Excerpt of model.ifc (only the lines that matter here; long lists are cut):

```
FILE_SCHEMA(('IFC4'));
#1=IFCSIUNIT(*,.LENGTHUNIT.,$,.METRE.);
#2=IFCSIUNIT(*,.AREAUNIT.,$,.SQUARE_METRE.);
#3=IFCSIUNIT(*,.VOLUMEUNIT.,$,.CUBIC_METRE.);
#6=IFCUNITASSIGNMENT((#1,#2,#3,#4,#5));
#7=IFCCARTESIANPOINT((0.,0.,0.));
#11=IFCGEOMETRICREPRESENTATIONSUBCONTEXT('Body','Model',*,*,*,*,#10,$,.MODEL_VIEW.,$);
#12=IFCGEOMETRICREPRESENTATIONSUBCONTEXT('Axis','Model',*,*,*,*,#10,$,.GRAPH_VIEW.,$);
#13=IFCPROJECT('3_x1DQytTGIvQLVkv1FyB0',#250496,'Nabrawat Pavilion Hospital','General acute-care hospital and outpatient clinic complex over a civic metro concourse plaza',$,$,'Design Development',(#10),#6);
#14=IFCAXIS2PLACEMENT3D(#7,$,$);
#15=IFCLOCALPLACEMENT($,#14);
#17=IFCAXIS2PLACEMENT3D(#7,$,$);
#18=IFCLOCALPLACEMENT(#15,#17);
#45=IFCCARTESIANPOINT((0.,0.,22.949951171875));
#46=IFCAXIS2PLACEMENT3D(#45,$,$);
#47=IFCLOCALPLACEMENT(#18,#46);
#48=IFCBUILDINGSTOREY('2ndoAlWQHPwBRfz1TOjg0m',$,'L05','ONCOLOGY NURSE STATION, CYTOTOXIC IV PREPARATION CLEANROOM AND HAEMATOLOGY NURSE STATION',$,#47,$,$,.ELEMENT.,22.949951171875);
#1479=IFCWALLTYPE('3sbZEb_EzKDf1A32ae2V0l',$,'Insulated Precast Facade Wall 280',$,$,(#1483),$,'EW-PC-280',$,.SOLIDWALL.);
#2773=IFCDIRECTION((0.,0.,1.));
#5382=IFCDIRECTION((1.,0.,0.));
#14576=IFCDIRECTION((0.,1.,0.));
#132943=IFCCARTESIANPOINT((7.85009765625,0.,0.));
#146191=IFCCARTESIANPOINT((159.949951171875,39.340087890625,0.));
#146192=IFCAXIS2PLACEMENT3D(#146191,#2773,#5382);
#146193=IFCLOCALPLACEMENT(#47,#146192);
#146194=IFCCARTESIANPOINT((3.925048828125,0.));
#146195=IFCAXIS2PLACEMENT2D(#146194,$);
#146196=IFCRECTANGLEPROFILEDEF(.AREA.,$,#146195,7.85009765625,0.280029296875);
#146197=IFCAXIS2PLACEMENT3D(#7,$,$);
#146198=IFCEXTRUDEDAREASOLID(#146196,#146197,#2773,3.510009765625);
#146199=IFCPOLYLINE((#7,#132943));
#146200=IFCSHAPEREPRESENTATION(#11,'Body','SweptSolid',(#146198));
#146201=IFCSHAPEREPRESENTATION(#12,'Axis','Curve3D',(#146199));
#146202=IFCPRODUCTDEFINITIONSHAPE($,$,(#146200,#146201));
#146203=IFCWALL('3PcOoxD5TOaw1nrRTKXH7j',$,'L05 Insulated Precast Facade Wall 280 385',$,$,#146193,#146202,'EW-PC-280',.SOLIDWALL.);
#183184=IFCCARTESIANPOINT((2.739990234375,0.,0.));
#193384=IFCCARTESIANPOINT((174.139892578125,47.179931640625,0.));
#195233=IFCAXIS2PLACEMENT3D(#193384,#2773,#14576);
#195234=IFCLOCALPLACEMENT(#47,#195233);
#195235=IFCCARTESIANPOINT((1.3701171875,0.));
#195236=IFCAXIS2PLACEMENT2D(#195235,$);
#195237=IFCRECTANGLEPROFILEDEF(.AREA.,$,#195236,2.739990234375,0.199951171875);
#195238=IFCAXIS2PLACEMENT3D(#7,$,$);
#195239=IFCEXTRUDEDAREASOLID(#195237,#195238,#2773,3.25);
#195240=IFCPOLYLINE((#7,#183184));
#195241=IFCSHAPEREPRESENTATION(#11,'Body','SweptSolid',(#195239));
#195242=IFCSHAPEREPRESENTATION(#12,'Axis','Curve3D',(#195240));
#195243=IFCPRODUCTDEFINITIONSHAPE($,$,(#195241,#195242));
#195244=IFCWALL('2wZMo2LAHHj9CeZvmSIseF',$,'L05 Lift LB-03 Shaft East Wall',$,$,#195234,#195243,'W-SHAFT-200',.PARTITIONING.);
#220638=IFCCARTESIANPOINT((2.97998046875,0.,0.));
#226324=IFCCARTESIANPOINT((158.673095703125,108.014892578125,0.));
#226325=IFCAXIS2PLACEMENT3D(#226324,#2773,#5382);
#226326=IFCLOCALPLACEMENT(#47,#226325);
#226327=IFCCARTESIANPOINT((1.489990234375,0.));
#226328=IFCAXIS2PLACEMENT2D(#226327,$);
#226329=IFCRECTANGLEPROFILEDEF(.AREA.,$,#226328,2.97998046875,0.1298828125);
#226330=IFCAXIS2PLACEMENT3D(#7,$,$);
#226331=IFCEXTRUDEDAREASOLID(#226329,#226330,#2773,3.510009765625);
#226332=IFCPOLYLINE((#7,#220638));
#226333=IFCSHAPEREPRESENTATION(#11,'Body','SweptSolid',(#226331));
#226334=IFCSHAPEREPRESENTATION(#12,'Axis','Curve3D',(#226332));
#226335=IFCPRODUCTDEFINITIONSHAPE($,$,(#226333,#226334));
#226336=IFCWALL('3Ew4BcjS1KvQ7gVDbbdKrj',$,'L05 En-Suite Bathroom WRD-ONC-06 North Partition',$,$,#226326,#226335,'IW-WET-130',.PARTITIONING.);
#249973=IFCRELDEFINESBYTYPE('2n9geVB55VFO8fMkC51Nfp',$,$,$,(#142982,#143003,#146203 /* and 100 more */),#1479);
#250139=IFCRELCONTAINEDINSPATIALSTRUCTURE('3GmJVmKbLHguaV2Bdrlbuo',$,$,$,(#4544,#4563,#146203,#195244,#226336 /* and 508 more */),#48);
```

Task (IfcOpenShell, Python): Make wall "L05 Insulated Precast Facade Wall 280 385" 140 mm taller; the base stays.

```python
import ifcopenshell
import ifcopenshell.geom
import ifcopenshell.util.representation
import ifcopenshell.util.shape
import ifcopenshell.util.unit

model = ifcopenshell.open("model.ifc")
unit_scale = ifcopenshell.util.unit.calculate_unit_scale(model)
settings = ifcopenshell.geom.settings()


def volume(element):
    """Net volume in cubic metres, openings subtracted."""
    shape = ifcopenshell.geom.create_shape(settings, element)
    return ifcopenshell.util.shape.get_volume(shape.geometry)


wall = model.by_guid("3PcOoxD5TOaw1nrRTKXH7j")
before = volume(wall)

body = ifcopenshell.util.representation.get_representation(wall, "Model", "Body")
solid = body.Items[0]
old_height = solid.Depth
solid.Depth += 0.14 / unit_scale
after = volume(wall)

print(f"height {old_height:g} -> {solid.Depth:g}, volume {before:.3f} -> {after:.3f} m3")

model.write("model_updated.ifc")
```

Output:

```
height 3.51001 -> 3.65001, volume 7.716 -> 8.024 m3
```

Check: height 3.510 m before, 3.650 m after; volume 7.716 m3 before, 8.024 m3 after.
